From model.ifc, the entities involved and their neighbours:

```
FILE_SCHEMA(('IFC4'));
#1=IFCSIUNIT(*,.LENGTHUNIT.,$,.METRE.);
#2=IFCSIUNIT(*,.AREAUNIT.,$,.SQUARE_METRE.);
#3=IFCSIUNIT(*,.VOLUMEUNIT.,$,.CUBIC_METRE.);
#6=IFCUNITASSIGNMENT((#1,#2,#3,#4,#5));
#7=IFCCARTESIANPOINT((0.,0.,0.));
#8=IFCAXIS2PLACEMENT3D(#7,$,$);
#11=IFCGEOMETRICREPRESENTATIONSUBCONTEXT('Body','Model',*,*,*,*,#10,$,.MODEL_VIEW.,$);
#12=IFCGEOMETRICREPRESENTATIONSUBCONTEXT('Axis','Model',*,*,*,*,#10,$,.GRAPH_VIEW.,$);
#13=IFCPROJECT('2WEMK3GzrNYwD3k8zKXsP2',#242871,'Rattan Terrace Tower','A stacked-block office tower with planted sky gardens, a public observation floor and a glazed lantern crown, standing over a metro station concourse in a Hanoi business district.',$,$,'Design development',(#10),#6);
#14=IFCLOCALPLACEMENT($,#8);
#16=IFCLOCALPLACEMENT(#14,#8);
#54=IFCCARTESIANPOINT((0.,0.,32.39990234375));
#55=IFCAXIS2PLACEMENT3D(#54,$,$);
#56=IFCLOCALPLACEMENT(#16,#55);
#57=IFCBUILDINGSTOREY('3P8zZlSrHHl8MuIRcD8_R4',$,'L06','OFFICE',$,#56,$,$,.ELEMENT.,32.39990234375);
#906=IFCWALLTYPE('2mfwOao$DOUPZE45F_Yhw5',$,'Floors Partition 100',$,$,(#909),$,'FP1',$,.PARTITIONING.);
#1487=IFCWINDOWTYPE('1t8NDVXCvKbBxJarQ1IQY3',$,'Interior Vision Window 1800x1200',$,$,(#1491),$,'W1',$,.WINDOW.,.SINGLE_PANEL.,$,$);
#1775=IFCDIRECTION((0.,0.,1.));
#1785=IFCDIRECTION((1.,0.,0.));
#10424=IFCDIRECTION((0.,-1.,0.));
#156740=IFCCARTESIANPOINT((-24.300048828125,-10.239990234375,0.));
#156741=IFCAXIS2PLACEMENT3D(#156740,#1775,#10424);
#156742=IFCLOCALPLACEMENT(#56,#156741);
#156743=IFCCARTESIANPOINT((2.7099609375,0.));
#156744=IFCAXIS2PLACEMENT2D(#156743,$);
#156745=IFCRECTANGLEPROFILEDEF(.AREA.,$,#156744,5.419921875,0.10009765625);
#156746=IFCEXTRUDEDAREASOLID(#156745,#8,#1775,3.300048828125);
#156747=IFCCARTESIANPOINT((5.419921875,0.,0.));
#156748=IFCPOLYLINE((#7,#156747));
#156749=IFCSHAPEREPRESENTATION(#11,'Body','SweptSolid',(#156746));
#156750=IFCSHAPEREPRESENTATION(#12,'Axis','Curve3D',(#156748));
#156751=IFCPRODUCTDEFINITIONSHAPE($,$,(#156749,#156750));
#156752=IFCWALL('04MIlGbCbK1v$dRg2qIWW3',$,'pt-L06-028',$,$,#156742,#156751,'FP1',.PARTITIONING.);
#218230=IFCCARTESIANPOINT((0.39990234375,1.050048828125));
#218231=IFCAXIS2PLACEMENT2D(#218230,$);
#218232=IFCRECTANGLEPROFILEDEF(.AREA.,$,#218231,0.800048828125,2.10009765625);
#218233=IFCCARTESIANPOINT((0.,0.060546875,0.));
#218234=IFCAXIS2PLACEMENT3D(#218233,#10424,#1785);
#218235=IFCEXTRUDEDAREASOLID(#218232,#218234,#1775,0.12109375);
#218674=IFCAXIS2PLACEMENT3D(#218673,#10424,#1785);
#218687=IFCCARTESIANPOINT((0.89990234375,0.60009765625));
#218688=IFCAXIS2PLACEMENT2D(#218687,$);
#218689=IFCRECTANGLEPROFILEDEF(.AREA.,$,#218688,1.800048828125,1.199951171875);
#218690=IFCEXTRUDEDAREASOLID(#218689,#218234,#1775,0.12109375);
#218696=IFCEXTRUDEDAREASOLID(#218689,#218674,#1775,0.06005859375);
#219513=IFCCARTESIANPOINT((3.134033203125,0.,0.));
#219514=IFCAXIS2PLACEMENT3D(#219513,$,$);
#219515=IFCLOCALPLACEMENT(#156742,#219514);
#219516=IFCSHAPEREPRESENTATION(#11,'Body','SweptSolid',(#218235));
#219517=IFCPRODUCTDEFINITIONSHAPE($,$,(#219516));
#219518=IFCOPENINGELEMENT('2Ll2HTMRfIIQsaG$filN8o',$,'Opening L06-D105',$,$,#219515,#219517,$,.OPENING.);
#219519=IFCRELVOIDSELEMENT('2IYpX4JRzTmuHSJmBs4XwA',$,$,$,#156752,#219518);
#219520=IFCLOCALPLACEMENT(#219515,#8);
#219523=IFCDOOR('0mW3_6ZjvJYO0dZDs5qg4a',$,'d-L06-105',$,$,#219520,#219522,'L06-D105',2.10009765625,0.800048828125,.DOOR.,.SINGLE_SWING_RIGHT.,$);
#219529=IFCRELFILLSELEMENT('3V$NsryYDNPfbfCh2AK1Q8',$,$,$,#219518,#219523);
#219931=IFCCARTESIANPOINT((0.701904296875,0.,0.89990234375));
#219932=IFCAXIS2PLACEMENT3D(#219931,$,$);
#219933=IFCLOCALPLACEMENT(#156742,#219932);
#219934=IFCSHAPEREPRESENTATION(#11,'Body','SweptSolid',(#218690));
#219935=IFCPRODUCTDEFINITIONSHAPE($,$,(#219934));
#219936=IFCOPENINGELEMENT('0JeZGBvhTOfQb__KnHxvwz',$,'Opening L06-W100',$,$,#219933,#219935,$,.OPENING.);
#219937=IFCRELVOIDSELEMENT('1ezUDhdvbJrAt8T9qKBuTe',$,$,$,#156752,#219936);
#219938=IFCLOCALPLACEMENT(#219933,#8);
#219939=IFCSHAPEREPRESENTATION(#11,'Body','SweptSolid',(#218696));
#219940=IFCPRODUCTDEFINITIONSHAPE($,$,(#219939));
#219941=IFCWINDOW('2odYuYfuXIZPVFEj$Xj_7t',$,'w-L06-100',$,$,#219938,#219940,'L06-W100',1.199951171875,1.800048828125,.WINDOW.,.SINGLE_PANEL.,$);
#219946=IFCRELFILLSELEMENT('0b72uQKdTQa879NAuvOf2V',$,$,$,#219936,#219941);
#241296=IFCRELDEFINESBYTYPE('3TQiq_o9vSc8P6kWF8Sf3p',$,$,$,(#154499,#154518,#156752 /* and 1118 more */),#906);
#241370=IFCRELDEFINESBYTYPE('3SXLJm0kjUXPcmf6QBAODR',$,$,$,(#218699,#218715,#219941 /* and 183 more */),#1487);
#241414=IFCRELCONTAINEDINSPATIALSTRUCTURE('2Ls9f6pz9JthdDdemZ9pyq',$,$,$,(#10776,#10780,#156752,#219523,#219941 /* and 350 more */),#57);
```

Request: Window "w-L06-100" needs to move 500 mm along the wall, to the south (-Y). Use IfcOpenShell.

```python
import ifcopenshell
import ifcopenshell.api.geometry
import ifcopenshell.util.placement

model = ifcopenshell.open("model.ifc")

window = model.by_guid("2odYuYfuXIZPVFEj$Xj_7t")
opening = window.FillsVoids[0].RelatingOpeningElement
wall = opening.VoidsElements[0].RelatingBuildingElement

wall_matrix = ifcopenshell.util.placement.get_local_placement(wall.ObjectPlacement)
shift = wall_matrix[:3, 0] * 0.5
before = ifcopenshell.util.placement.get_local_placement(window.ObjectPlacement)[:3, 3].copy()

# The window is placed relative to its opening, so it follows when the opening moves.
matrix = ifcopenshell.util.placement.get_local_placement(opening.ObjectPlacement)
matrix[:3, 3] += shift
ifcopenshell.api.geometry.edit_object_placement(
    model, product=opening, matrix=matrix, is_si=False, should_transform_children=True
)

after = ifcopenshell.util.placement.get_local_placement(window.ObjectPlacement)[:3, 3]
print("window moved by", (after - before).round(3) + 0.0)

model.write("model_updated.ifc")
```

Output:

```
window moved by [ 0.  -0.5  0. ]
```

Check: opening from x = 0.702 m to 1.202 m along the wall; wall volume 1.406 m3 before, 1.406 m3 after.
